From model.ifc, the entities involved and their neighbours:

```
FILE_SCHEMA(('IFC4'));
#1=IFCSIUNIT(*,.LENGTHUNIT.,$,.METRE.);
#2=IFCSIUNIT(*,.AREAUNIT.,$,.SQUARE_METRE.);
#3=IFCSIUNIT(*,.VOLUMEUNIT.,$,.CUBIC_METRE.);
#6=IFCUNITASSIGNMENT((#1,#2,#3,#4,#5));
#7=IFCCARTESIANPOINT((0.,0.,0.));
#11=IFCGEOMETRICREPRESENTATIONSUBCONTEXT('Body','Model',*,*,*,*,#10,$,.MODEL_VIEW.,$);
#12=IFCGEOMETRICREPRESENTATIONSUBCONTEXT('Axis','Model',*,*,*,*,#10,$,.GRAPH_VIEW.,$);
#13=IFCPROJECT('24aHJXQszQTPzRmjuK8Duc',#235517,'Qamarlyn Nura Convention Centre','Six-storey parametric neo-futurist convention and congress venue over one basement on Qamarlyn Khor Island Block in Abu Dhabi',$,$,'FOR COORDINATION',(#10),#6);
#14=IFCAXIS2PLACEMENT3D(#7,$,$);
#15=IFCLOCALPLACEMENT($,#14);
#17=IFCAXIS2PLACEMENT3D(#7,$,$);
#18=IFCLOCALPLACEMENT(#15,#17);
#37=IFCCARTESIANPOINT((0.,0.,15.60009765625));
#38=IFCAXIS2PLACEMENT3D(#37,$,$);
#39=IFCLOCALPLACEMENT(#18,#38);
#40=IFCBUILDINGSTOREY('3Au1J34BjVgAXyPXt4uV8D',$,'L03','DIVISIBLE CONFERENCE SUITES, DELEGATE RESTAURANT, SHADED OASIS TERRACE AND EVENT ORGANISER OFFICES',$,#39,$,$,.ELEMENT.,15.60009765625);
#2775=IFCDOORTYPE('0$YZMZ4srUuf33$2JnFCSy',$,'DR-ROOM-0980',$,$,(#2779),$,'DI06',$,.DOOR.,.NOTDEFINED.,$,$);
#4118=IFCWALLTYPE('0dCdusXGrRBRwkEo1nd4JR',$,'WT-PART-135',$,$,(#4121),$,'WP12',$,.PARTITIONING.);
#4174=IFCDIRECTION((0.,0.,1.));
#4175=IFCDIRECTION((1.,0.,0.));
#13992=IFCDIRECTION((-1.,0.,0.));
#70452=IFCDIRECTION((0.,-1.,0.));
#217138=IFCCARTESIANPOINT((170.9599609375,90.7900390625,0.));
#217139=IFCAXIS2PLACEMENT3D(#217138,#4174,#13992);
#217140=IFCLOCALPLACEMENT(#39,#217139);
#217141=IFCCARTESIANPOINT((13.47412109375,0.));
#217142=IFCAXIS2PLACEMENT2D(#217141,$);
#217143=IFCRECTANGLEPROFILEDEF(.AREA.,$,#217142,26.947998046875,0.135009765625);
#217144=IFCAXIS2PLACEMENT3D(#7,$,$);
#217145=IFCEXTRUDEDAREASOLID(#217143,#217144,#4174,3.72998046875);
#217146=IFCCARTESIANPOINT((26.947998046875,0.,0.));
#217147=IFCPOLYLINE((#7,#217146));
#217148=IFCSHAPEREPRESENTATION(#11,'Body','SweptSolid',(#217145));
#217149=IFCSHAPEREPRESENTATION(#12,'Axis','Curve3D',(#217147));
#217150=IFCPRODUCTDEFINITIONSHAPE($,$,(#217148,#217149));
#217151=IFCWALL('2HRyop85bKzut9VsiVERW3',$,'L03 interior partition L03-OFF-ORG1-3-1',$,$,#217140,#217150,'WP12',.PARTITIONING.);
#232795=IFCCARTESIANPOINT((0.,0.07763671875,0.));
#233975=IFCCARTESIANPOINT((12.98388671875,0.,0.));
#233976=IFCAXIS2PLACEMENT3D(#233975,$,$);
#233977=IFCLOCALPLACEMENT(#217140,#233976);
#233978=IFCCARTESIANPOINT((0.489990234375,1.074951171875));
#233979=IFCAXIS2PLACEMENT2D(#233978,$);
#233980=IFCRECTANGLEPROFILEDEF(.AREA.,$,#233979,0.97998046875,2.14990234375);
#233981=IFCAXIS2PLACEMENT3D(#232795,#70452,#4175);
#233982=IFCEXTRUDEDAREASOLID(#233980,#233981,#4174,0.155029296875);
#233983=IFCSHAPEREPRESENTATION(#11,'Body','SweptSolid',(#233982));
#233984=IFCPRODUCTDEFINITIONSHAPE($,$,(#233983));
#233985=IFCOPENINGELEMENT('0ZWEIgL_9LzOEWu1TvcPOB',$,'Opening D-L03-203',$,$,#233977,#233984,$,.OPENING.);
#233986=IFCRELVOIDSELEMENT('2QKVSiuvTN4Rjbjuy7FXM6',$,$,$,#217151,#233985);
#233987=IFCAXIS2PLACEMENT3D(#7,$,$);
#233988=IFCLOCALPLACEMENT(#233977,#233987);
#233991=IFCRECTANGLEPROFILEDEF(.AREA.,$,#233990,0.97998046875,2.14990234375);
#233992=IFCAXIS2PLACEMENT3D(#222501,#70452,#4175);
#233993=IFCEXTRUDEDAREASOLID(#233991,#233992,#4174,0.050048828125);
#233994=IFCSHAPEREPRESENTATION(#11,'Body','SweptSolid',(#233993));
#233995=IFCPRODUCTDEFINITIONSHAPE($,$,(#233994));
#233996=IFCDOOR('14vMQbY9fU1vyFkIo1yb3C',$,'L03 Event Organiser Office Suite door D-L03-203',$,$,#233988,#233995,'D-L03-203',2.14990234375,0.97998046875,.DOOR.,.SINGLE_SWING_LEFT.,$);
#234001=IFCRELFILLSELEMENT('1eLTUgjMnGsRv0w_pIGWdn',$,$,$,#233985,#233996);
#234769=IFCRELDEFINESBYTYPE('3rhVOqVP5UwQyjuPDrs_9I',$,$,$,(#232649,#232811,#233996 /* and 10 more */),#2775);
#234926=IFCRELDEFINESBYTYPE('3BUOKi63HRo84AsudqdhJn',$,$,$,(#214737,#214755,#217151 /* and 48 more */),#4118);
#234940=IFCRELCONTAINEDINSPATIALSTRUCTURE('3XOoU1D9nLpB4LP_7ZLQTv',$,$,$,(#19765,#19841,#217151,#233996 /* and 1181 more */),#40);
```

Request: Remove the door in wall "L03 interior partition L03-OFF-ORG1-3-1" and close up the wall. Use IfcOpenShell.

```python
import ifcopenshell
import ifcopenshell.api.feature
import ifcopenshell.api.root
import ifcopenshell.geom
import ifcopenshell.util.shape

model = ifcopenshell.open("model.ifc")
settings = ifcopenshell.geom.settings()


def volume(element):
    """Net volume in cubic metres, openings subtracted."""
    shape = ifcopenshell.geom.create_shape(settings, element)
    return ifcopenshell.util.shape.get_volume(shape.geometry)


door = model.by_id(233996)
opening = door.FillsVoids[0].RelatingOpeningElement
wall = opening.VoidsElements[0].RelatingBuildingElement
before = volume(wall)

ifcopenshell.api.root.remove_product(model, product=door)
ifcopenshell.api.feature.remove_feature(model, feature=opening)

after = volume(wall)

print(f"wall volume {before:.3f} -> {after:.3f} m3")

model.write("model_edited.ifc")
```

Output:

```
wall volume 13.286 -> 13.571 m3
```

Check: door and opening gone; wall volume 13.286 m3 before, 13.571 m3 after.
